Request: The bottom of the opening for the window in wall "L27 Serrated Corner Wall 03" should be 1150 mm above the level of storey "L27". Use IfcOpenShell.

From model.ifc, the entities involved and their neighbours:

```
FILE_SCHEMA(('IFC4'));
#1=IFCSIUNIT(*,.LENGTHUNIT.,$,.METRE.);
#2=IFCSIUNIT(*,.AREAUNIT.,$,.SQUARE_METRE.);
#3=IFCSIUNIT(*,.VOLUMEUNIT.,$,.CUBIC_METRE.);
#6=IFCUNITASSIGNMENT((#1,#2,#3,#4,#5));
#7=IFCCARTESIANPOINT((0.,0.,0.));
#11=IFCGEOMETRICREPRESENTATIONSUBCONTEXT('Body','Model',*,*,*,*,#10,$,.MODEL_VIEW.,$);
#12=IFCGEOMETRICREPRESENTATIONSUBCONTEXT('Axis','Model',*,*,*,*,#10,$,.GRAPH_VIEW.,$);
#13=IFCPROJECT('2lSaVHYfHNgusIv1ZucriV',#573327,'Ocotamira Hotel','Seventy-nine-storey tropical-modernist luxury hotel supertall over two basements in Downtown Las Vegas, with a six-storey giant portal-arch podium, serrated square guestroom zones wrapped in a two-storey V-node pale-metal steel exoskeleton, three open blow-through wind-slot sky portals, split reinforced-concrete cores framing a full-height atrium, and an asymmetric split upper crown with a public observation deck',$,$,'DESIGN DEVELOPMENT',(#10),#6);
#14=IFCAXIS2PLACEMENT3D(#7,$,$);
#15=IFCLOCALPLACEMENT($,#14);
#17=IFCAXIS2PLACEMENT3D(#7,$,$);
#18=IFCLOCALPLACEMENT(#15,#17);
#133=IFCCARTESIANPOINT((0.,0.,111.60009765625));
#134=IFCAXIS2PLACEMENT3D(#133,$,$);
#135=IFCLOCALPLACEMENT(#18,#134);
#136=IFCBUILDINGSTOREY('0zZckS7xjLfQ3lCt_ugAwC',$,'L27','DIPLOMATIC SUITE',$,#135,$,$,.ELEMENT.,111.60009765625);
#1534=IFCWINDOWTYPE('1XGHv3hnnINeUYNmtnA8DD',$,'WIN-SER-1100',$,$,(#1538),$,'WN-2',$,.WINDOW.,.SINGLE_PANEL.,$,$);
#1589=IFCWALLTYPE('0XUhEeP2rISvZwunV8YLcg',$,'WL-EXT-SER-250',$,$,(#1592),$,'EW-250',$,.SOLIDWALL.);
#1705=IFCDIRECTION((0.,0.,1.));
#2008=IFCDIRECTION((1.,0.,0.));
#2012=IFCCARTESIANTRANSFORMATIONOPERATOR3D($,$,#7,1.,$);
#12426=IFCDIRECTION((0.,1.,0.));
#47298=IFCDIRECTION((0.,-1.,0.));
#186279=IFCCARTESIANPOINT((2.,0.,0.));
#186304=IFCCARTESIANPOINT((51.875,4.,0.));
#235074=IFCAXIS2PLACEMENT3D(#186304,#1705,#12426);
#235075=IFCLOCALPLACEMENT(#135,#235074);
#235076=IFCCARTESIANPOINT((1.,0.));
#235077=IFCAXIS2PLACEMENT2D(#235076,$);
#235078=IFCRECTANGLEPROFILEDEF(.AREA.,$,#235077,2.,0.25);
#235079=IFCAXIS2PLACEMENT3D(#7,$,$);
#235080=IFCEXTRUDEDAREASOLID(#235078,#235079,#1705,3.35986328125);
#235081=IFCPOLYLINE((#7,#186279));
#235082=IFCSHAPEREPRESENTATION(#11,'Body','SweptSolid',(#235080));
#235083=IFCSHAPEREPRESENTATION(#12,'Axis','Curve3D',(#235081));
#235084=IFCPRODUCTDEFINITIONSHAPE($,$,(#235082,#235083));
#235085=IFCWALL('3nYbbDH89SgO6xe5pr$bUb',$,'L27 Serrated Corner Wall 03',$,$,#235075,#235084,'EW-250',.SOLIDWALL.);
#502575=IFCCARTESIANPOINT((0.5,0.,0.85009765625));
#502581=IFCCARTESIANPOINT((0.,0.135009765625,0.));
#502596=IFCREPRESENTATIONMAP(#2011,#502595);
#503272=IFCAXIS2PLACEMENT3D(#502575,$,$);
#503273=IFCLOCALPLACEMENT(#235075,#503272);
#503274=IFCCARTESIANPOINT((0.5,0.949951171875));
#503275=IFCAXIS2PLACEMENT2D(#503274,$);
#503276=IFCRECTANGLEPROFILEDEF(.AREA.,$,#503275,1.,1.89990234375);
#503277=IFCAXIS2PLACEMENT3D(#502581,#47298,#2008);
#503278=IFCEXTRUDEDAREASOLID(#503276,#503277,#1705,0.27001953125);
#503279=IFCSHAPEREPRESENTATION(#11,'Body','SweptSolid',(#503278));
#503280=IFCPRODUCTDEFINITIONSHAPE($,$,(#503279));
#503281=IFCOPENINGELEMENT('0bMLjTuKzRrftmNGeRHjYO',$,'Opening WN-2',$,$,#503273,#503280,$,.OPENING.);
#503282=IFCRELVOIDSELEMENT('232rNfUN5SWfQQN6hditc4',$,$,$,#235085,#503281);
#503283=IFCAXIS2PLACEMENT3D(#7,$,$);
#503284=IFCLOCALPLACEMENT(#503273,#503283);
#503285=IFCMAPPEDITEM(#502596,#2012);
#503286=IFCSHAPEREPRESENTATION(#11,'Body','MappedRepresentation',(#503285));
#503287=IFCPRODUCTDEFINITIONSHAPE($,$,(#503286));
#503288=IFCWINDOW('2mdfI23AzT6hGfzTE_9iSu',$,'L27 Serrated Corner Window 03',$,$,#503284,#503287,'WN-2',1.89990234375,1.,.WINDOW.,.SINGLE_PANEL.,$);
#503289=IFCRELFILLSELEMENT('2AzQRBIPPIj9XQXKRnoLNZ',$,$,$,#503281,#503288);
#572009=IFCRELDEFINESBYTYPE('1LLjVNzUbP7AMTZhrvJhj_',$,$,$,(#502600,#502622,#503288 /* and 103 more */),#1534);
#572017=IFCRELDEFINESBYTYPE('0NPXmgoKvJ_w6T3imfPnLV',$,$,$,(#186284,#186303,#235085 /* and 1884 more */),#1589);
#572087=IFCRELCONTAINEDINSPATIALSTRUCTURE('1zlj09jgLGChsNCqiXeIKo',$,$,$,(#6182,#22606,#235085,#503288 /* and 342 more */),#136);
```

```python
import numpy as np
import ifcopenshell
import ifcopenshell.api.geometry
import ifcopenshell.geom
import ifcopenshell.util.element
import ifcopenshell.util.placement
import ifcopenshell.util.shape
import ifcopenshell.util.unit

model = ifcopenshell.open("model.ifc")
unit_scale = ifcopenshell.util.unit.calculate_unit_scale(model)

window = model.by_guid("2mdfI23AzT6hGfzTE_9iSu")
opening = window.FillsVoids[0].RelatingOpeningElement
storey = ifcopenshell.util.element.get_container(window, ifc_class="IfcBuildingStorey")
level = ifcopenshell.util.placement.get_local_placement(storey.ObjectPlacement)[2, 3]

# The opening's origin need not be at the sill, so measure its lowest point.
shape = ifcopenshell.geom.create_shape(ifcopenshell.geom.settings(), opening)
bottom = ifcopenshell.util.shape.get_shape_bottom_elevation(shape, shape.geometry) / unit_scale
dz = level + 1.15 / unit_scale - bottom

shift = np.array([0.0, 0.0, dz])
# The window is placed relative to its opening, so it follows when the opening moves.
matrix = ifcopenshell.util.placement.get_local_placement(opening.ObjectPlacement)
matrix[:3, 3] += shift
ifcopenshell.api.geometry.edit_object_placement(
    model, product=opening, matrix=matrix, is_si=False, should_transform_children=True
)

print(f"moved by {dz * unit_scale:+.3f} m")

model.write("model_v2.ifc")
```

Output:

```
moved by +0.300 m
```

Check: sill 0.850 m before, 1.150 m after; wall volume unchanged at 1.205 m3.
